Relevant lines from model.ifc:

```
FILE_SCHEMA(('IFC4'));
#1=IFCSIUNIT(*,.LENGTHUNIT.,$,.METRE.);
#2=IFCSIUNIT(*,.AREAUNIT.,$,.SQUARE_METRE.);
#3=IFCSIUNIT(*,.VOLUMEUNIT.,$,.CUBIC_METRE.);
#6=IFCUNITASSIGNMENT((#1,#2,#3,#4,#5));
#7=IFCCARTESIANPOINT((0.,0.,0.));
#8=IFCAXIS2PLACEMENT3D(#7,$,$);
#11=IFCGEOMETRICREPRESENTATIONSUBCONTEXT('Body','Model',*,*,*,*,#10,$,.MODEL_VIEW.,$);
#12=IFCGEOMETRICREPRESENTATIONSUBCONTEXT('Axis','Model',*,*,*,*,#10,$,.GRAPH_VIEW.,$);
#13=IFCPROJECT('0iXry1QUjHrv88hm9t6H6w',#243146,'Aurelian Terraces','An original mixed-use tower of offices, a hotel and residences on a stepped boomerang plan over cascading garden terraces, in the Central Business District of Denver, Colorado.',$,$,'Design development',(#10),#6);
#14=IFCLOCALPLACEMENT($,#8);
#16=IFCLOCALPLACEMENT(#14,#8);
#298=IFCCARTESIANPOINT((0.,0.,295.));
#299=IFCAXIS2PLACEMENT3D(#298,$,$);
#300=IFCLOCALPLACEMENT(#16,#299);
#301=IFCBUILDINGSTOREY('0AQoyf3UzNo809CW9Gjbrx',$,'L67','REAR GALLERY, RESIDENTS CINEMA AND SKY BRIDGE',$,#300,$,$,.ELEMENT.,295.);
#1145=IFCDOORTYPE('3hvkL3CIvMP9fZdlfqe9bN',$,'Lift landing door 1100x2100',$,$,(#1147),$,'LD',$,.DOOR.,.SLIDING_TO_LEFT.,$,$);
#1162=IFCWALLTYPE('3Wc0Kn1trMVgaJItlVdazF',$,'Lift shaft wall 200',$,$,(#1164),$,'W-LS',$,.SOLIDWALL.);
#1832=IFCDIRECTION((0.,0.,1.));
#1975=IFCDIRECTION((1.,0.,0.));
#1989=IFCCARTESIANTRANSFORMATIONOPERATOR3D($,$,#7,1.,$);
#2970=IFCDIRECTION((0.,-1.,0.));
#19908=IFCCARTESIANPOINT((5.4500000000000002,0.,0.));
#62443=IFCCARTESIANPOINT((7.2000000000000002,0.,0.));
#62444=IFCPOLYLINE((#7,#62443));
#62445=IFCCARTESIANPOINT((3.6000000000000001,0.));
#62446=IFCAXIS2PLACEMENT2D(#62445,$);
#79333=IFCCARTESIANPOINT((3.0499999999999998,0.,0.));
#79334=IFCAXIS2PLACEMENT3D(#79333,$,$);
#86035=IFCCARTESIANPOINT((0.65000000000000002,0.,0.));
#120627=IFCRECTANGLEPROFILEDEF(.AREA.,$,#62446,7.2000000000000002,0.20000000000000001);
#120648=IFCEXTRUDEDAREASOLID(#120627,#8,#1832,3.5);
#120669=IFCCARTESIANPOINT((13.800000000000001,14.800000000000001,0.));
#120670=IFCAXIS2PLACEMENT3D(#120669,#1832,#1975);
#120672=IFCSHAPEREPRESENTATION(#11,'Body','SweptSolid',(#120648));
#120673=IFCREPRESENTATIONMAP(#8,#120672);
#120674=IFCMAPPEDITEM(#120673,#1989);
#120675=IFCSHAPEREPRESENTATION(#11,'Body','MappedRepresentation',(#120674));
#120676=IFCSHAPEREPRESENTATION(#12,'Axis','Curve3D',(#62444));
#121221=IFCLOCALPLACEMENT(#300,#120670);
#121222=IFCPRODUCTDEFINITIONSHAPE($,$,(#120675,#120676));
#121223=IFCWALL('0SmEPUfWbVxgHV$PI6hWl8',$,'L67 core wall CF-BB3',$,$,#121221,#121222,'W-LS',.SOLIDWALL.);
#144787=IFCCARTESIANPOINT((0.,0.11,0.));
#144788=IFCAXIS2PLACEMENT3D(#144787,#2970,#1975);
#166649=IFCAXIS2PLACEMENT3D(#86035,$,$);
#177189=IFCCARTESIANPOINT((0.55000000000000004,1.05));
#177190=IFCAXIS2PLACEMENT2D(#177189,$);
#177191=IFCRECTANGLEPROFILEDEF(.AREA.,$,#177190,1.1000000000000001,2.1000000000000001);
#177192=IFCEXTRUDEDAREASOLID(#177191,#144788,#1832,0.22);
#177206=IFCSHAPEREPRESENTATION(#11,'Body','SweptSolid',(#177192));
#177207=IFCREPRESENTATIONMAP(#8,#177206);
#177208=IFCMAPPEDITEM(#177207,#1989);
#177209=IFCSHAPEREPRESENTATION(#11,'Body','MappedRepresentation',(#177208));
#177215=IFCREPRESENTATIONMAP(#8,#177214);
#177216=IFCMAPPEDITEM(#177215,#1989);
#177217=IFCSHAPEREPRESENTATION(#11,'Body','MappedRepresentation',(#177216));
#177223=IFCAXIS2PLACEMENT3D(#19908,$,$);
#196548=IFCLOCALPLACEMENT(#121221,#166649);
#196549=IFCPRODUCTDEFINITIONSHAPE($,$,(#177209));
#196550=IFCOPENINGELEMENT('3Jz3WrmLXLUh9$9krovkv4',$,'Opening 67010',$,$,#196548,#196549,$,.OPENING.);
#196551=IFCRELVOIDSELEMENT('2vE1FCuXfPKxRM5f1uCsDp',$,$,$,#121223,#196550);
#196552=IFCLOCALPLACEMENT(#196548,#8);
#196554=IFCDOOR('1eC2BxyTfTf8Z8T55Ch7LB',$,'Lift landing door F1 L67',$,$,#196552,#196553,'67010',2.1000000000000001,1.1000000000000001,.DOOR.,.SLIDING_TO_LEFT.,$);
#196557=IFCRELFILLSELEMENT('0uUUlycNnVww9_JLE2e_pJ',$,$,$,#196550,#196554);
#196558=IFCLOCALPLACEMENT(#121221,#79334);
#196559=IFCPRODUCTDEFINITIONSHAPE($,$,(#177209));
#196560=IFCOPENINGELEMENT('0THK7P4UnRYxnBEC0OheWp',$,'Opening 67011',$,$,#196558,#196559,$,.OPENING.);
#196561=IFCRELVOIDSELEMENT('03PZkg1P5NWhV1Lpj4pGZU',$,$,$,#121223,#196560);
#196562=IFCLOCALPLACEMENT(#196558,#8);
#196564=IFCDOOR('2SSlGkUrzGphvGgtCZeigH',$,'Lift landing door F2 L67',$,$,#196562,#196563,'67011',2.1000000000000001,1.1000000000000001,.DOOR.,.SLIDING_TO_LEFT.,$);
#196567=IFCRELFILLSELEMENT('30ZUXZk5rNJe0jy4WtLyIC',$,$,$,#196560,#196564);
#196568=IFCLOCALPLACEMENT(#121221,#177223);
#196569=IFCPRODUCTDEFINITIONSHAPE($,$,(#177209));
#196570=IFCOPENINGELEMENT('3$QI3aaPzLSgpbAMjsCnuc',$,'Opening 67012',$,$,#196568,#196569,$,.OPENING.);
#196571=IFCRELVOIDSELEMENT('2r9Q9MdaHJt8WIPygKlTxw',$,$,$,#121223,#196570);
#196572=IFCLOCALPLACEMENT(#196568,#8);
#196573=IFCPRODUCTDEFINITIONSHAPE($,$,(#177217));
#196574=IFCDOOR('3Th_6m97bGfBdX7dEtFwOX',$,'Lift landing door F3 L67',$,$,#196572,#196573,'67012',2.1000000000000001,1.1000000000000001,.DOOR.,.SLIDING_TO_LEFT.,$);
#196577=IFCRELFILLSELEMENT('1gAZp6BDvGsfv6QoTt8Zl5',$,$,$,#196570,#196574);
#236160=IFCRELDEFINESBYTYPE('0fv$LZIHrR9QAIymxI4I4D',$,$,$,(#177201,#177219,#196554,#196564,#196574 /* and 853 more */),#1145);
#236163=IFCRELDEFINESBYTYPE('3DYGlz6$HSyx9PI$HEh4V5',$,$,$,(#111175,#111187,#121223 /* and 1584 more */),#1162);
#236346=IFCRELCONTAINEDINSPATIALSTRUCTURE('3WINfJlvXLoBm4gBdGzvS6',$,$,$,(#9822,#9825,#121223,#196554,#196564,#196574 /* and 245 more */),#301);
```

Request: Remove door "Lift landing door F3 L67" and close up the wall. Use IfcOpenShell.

```python
import ifcopenshell
import ifcopenshell.api.feature
import ifcopenshell.api.root
import ifcopenshell.geom
import ifcopenshell.util.shape

model = ifcopenshell.open("model.ifc")
settings = ifcopenshell.geom.settings()


def volume(element):
    """Net volume in cubic metres, openings subtracted."""
    shape = ifcopenshell.geom.create_shape(settings, element)
    return ifcopenshell.util.shape.get_volume(shape.geometry)


door = model.by_guid("3Th_6m97bGfBdX7dEtFwOX")
opening = door.FillsVoids[0].RelatingOpeningElement
wall = opening.VoidsElements[0].RelatingBuildingElement
before = volume(wall)

ifcopenshell.api.root.remove_product(model, product=door)
ifcopenshell.api.feature.remove_feature(model, feature=opening)

after = volume(wall)

print(f"wall volume {before:.3f} -> {after:.3f} m3")

model.write("model_v2.ifc")
```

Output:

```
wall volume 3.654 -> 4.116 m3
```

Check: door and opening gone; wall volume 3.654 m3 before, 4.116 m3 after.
